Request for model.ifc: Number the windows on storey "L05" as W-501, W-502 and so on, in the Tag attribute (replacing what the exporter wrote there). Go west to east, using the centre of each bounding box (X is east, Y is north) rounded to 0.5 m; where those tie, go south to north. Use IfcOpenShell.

First a look at what the model holds.

```python
import ifcopenshell
import ifcopenshell.util.element
import ifcopenshell.util.placement

model = ifcopenshell.open("model.ifc")
print(model.schema)
storey = next(s for s in model.by_type("IfcBuildingStorey") if s.Name == "L05")
windows = [e for e in ifcopenshell.util.element.get_decomposition(storey) if e.is_a("IfcWindow")]
for e in sorted(windows, key=lambda e: e.id()):
    origin = ifcopenshell.util.placement.get_local_placement(e.ObjectPlacement)[:3, 3]
    print(e.id(), e.Tag, e.Name, origin.round(2) + 0.0, sep=" | ")
```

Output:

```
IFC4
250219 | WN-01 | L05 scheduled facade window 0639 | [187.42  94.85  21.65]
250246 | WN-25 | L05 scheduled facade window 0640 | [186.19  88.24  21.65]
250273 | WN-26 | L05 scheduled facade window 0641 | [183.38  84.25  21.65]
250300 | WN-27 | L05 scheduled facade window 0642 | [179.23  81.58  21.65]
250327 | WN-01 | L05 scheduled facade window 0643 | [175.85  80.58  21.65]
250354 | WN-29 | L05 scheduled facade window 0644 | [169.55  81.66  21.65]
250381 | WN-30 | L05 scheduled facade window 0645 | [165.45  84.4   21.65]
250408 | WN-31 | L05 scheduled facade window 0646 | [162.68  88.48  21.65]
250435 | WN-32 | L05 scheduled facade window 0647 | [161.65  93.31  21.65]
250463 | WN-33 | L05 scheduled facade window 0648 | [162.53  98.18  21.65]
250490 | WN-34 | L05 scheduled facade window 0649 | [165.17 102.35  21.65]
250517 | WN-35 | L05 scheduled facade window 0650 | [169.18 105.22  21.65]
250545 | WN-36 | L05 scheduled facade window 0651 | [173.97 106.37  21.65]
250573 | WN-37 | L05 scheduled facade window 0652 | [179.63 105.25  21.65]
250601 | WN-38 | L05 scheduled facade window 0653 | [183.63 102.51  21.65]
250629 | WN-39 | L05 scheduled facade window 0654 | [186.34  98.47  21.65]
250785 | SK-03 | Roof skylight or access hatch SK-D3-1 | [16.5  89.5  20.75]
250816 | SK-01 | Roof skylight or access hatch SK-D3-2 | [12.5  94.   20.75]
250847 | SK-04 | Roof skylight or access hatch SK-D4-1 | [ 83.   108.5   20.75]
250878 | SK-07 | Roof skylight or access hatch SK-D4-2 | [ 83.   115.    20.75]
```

```python
import ifcopenshell
import ifcopenshell.geom
import ifcopenshell.util.element
import ifcopenshell.util.shape

model = ifcopenshell.open("model.ifc")
settings = ifcopenshell.geom.settings()
settings.set("use-world-coords", True)


def centre(element):
    shape = ifcopenshell.geom.create_shape(settings, element)
    return ifcopenshell.util.shape.get_bbox_centroid(shape.geometry)


storey = next(s for s in model.by_type("IfcBuildingStorey") if s.Name == "L05")
windows = [e for e in ifcopenshell.util.element.get_decomposition(storey) if e.is_a("IfcWindow")]

# Insertion points can sit at a corner or the storey origin, so sort by the geometry (in metres).
centres = {e: centre(e) for e in windows}
windows.sort(key=lambda e: (round(centres[e][0] / 0.5), centres[e][1]))

for i, e in enumerate(windows, start=1):
    number = f"W-5{i:02d}"
    e.Tag = number
    print(e.id(), number)

model.write("model-out.ifc")
```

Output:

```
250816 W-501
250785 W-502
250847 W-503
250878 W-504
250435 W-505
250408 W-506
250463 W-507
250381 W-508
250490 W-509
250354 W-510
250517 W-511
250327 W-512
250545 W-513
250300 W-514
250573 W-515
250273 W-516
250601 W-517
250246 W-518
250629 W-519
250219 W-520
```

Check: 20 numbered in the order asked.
